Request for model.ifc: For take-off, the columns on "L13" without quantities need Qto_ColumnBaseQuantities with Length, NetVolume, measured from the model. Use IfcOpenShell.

First a look at what the model holds.

```python
import ifcopenshell
import ifcopenshell.util.element
import ifcopenshell.util.unit

model = ifcopenshell.open("model.ifc")
print(model.schema)
for unit_type in ("LENGTHUNIT", "AREAUNIT", "VOLUMEUNIT"):
    print(unit_type, ifcopenshell.util.unit.calculate_unit_scale(model, unit_type))
storey = next(s for s in model.by_type("IfcBuildingStorey") if s.Name == "L13")
columns = [e for e in ifcopenshell.util.element.get_decomposition(storey) if e.is_a("IfcColumn")]
for e in sorted(columns, key=lambda e: e.id()):
    print(e.id(), e.is_a(), e.Name, list(ifcopenshell.util.element.get_psets(e, qtos_only=True)), sep=" | ")
```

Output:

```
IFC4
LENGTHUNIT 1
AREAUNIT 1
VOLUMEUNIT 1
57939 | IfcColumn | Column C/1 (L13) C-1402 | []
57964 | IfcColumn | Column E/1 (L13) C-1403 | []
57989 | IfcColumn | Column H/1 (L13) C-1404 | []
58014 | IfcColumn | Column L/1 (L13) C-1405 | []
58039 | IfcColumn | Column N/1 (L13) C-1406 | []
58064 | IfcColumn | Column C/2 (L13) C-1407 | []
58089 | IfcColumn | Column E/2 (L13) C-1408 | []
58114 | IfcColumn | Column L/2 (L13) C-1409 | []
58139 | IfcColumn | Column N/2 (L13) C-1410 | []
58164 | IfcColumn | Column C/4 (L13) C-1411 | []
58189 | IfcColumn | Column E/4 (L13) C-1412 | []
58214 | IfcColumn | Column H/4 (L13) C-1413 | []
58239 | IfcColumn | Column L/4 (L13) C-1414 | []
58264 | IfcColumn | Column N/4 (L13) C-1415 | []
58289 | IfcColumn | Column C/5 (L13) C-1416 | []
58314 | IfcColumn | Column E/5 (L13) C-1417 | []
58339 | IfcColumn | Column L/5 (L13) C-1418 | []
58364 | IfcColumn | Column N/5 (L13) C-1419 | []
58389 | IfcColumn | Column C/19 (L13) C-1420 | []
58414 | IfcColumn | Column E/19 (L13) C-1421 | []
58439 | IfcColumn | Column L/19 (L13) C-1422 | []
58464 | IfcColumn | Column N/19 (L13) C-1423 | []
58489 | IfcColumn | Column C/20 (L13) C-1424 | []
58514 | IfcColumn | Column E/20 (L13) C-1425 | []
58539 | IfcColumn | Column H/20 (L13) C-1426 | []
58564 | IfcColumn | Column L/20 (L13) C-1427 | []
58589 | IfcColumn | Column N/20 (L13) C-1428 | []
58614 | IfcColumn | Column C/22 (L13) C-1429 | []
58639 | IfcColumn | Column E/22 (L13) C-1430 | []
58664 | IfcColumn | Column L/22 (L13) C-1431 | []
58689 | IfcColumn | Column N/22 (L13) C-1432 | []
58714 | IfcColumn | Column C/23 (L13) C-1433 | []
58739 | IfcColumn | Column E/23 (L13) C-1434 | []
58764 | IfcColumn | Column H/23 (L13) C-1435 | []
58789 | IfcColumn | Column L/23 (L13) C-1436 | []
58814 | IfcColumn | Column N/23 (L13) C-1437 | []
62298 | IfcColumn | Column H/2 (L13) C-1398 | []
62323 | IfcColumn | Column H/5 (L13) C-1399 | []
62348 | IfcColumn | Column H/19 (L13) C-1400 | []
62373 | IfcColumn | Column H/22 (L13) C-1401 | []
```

```python
import ifcopenshell
import ifcopenshell.api.pset
import ifcopenshell.geom
import ifcopenshell.util.element
import ifcopenshell.util.shape
import ifcopenshell.util.unit

model = ifcopenshell.open("model.ifc")
unit_scale = ifcopenshell.util.unit.calculate_unit_scale(model)
volume_scale = ifcopenshell.util.unit.calculate_unit_scale(model, "VOLUMEUNIT")
settings = ifcopenshell.geom.settings()

storey = next(s for s in model.by_type("IfcBuildingStorey") if s.Name == "L13")
columns = [e for e in ifcopenshell.util.element.get_decomposition(storey) if e.is_a("IfcColumn")]

for e in sorted(columns, key=lambda e: e.id()):
    if ifcopenshell.util.element.get_psets(e, qtos_only=True, should_inherit=False):
        continue
    # Geometry comes back in metres, in the element's own axes.
    shape = ifcopenshell.geom.create_shape(settings, e)
    values = {
        "Length": ifcopenshell.util.shape.get_z(shape.geometry) / unit_scale,
        "NetVolume": ifcopenshell.util.shape.get_volume(shape.geometry) / volume_scale,
    }
    qto = ifcopenshell.api.pset.add_qto(model, product=e, name="Qto_ColumnBaseQuantities")
    ifcopenshell.api.pset.edit_qto(model, qto=qto, properties=values)
    print(e.id(), {k: round(v, 3) for k, v in values.items()})

model.write("model-out.ifc")
```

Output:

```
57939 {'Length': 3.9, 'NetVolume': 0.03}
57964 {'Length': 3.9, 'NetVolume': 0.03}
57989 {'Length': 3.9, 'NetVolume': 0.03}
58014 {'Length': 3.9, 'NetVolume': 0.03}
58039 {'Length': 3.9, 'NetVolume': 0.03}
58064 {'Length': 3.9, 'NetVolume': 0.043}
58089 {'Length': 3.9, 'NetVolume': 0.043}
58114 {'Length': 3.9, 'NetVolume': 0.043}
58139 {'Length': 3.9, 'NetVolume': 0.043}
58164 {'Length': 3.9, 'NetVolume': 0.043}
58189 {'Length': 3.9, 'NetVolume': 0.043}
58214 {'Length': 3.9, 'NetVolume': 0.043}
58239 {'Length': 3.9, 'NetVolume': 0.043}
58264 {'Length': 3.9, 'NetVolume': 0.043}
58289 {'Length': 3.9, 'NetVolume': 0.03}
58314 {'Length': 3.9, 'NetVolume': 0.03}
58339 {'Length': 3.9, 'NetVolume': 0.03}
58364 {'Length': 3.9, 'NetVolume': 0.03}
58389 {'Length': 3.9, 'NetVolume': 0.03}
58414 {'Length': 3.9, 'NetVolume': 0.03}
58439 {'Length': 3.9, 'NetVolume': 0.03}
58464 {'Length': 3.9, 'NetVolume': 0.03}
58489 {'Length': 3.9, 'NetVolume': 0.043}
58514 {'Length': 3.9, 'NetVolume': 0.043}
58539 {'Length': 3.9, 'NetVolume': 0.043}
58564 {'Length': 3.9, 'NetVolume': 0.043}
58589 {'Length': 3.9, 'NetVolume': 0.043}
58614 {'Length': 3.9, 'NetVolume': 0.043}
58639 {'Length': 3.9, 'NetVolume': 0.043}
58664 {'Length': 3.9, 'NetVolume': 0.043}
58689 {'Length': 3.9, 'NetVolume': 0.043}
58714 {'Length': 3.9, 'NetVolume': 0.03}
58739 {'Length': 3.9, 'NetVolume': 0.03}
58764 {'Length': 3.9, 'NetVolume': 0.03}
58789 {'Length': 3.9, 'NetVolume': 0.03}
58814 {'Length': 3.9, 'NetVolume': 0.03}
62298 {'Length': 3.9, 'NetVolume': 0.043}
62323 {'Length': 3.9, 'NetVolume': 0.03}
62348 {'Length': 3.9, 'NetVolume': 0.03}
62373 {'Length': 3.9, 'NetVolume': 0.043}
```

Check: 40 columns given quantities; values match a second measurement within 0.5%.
